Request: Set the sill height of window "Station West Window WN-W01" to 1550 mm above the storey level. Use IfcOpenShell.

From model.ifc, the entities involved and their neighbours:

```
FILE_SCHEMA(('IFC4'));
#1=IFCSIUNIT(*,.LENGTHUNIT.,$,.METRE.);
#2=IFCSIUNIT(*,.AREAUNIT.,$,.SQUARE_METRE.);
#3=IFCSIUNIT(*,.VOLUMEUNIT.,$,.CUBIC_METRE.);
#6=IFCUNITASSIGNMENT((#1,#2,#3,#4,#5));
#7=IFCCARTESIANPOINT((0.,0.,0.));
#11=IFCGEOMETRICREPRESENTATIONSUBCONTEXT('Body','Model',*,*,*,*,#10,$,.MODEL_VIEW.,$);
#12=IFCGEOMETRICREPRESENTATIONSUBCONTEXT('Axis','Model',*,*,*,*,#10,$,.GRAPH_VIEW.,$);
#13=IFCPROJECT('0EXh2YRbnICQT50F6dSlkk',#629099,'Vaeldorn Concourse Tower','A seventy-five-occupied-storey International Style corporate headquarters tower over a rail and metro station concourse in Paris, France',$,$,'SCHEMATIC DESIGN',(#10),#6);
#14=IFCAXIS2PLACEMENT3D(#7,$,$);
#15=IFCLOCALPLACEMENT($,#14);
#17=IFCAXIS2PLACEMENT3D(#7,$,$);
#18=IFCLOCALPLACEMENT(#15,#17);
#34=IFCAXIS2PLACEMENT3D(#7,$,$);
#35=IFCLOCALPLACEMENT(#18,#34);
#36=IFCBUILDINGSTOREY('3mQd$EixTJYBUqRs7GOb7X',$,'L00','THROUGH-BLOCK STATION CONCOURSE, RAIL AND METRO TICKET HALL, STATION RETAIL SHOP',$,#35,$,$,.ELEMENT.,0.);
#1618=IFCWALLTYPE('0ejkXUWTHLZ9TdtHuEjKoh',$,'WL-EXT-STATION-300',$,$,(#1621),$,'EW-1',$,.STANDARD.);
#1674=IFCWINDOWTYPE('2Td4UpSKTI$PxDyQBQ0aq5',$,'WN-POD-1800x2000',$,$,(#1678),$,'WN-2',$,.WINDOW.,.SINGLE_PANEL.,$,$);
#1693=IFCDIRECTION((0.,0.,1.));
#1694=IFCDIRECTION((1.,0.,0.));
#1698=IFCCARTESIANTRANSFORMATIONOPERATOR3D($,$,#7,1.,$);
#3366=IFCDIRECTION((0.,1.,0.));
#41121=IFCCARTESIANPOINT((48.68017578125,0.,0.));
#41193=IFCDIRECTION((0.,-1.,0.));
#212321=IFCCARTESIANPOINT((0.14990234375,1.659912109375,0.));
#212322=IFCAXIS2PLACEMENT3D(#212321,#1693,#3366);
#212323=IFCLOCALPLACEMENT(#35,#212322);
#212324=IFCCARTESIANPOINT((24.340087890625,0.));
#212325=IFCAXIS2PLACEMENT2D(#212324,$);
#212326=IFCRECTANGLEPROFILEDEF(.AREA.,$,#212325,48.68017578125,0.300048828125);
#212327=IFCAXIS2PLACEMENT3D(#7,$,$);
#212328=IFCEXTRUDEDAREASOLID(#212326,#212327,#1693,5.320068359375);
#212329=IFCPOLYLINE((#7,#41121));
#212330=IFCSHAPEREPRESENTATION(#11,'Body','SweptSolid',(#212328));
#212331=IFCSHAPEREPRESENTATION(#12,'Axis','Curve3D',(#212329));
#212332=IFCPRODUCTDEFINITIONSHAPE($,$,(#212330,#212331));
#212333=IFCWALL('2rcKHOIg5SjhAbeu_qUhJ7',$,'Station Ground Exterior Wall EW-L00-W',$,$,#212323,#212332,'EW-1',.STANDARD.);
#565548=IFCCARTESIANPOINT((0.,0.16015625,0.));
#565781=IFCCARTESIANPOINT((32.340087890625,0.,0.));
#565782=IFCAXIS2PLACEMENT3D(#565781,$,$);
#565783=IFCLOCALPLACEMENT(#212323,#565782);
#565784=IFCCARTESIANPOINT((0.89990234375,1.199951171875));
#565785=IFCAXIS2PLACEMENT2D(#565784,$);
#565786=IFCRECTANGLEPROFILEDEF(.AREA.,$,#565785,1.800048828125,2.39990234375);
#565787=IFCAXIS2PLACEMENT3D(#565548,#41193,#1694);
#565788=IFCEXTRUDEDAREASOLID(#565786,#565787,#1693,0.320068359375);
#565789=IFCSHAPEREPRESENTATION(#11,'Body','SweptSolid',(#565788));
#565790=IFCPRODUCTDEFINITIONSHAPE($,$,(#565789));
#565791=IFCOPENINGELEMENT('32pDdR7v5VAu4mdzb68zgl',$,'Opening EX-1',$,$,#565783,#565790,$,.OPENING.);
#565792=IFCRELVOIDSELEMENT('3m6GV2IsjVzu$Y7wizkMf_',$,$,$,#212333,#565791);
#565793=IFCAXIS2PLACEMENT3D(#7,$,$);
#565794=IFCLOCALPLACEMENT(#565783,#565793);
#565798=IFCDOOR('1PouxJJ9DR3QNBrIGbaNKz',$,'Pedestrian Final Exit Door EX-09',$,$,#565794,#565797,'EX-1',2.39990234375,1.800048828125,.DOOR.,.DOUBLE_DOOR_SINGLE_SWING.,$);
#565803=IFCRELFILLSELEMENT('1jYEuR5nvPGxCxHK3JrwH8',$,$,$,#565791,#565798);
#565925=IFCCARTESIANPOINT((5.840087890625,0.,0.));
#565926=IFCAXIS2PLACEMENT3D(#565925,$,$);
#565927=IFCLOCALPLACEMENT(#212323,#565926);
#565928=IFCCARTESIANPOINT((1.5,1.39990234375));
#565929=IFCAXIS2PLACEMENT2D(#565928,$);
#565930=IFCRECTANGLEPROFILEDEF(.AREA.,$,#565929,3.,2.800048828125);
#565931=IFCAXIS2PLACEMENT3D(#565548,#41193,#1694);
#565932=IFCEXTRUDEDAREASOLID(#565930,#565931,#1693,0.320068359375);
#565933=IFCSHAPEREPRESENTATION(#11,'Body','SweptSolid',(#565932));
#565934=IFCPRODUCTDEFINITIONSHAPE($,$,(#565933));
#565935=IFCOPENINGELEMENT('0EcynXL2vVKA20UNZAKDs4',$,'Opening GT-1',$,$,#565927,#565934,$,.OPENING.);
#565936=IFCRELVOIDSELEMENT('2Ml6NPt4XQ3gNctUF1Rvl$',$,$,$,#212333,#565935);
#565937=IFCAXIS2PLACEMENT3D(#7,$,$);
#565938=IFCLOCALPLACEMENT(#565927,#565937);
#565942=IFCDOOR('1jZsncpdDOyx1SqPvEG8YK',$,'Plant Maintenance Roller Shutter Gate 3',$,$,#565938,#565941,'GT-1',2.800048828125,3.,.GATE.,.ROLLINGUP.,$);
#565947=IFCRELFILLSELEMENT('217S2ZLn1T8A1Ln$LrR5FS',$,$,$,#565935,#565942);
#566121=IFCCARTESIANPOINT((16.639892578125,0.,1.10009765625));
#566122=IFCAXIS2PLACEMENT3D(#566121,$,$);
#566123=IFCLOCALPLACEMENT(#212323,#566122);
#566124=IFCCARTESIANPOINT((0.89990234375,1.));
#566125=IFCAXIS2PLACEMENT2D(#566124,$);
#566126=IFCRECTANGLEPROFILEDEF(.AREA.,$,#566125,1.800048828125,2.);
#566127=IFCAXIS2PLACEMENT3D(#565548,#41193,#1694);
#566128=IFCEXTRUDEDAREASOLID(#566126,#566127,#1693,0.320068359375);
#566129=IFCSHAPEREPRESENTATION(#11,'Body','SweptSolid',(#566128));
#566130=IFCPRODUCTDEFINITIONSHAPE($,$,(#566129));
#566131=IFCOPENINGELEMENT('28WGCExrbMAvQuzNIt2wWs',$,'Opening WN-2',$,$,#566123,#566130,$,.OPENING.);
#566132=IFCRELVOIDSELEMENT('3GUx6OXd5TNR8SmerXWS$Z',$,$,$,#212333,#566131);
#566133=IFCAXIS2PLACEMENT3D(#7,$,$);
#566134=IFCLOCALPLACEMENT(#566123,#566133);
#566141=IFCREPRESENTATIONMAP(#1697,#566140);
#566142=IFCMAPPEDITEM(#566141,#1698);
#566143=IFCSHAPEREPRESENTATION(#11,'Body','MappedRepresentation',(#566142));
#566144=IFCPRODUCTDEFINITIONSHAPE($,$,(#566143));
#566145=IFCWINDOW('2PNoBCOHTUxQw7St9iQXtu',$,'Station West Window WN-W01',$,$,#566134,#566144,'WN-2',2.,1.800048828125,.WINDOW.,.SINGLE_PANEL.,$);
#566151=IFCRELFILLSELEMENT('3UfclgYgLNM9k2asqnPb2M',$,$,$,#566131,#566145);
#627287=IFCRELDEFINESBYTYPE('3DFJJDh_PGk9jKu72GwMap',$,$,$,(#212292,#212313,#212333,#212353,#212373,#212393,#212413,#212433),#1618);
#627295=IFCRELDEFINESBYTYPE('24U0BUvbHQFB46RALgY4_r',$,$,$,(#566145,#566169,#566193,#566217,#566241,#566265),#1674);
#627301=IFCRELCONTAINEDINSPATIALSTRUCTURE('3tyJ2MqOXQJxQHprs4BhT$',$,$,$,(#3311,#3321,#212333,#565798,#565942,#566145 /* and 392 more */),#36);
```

```python
import numpy as np
import ifcopenshell
import ifcopenshell.api.geometry
import ifcopenshell.geom
import ifcopenshell.util.element
import ifcopenshell.util.placement
import ifcopenshell.util.shape
import ifcopenshell.util.unit

model = ifcopenshell.open("model.ifc")
unit_scale = ifcopenshell.util.unit.calculate_unit_scale(model)

window = model.by_guid("2PNoBCOHTUxQw7St9iQXtu")
opening = window.FillsVoids[0].RelatingOpeningElement
storey = ifcopenshell.util.element.get_container(window, ifc_class="IfcBuildingStorey")
level = ifcopenshell.util.placement.get_local_placement(storey.ObjectPlacement)[2, 3]

# The opening's origin need not be at the sill, so measure its lowest point.
shape = ifcopenshell.geom.create_shape(ifcopenshell.geom.settings(), opening)
bottom = ifcopenshell.util.shape.get_shape_bottom_elevation(shape, shape.geometry) / unit_scale
dz = level + 1.55 / unit_scale - bottom

shift = np.array([0.0, 0.0, dz])
# The window is placed relative to its opening, so it follows when the opening moves.
matrix = ifcopenshell.util.placement.get_local_placement(opening.ObjectPlacement)
matrix[:3, 3] += shift
ifcopenshell.api.geometry.edit_object_placement(
    model, product=opening, matrix=matrix, is_si=False, should_transform_children=True
)

print(f"moved by {dz * unit_scale:+.3f} m")

model.write("model-out.ifc")
```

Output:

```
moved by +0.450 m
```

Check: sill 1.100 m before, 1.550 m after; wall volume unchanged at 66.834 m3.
